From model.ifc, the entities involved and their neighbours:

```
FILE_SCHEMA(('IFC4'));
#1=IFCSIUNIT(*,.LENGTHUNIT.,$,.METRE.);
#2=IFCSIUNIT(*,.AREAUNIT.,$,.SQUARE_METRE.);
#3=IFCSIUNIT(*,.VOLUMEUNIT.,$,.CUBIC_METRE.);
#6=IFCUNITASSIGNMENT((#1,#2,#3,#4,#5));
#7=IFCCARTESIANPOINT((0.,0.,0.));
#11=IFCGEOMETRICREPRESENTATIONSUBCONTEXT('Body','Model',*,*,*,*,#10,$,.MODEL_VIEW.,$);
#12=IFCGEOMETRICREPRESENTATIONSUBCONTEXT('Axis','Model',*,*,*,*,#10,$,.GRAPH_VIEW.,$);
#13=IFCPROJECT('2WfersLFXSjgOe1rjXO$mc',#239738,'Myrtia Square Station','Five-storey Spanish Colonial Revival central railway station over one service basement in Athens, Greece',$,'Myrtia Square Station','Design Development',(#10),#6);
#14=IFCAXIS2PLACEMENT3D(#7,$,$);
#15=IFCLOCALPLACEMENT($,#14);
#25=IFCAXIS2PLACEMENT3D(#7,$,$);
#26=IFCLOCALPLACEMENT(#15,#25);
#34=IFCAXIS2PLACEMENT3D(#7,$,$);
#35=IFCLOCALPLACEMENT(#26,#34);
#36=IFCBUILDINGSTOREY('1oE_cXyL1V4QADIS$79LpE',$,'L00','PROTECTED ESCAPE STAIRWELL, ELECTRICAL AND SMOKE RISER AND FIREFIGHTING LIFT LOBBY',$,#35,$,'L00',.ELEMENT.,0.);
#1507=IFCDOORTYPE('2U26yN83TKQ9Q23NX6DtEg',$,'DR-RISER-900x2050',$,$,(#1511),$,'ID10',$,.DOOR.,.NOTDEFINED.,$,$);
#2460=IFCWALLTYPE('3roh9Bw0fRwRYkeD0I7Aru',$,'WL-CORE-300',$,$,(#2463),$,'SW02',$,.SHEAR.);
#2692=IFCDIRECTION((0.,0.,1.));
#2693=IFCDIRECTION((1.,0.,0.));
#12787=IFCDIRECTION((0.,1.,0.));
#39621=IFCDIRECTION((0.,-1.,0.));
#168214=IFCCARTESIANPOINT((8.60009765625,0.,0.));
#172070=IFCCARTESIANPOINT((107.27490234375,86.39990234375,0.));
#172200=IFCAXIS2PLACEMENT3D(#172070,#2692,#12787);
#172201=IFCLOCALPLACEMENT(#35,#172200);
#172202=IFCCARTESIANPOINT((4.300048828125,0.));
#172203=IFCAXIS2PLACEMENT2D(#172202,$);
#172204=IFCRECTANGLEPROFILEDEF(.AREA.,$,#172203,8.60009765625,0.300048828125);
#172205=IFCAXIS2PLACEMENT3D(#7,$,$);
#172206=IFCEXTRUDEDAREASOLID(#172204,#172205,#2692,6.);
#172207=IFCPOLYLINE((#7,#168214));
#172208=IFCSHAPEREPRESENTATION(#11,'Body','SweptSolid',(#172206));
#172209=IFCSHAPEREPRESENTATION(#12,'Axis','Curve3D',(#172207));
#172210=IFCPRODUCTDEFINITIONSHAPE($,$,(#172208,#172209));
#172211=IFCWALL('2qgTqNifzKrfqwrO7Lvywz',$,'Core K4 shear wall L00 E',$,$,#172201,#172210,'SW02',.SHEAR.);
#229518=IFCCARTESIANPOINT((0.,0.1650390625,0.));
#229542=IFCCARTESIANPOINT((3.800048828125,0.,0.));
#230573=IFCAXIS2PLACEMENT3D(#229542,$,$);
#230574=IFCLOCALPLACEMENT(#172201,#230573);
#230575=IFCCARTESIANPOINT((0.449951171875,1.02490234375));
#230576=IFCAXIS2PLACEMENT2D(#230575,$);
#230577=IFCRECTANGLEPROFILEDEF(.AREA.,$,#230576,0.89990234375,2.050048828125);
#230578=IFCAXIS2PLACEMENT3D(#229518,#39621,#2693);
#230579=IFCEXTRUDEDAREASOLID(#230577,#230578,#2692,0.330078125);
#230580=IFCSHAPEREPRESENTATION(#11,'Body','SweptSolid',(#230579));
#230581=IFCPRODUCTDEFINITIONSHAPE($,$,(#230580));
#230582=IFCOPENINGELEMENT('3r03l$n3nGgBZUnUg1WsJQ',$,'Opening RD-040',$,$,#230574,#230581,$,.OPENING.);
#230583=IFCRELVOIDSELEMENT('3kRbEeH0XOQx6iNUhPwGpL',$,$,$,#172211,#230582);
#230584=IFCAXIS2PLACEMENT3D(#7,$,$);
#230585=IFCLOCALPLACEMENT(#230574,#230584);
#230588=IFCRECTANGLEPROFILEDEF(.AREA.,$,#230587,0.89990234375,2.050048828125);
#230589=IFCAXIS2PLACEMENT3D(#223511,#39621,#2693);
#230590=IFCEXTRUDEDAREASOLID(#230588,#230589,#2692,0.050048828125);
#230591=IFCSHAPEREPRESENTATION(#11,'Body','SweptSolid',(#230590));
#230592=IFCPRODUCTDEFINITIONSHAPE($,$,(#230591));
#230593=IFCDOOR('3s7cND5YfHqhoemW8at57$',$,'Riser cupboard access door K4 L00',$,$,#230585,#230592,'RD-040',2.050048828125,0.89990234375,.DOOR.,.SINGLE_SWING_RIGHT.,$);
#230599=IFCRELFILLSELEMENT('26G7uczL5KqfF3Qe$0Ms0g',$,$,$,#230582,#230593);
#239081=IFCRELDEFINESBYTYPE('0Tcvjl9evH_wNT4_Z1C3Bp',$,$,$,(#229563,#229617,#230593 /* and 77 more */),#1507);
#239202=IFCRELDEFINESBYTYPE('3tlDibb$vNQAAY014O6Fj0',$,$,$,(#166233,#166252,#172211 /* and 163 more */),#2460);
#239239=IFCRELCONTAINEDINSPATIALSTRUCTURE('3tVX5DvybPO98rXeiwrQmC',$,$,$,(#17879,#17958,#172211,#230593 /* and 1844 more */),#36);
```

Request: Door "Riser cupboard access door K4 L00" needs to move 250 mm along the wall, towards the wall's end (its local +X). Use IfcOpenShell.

```python
import ifcopenshell
import ifcopenshell.api.geometry
import ifcopenshell.util.placement
import ifcopenshell.util.unit

model = ifcopenshell.open("model.ifc")
unit_scale = ifcopenshell.util.unit.calculate_unit_scale(model)

door = model.by_id(230593)
opening = door.FillsVoids[0].RelatingOpeningElement
wall = opening.VoidsElements[0].RelatingBuildingElement

wall_matrix = ifcopenshell.util.placement.get_local_placement(wall.ObjectPlacement)
shift = wall_matrix[:3, 0] * 0.25 / unit_scale
before = ifcopenshell.util.placement.get_local_placement(door.ObjectPlacement)[:3, 3].copy()

# The door is placed relative to its opening, so it follows when the opening moves.
matrix = ifcopenshell.util.placement.get_local_placement(opening.ObjectPlacement)
matrix[:3, 3] += shift
ifcopenshell.api.geometry.edit_object_placement(
    model, product=opening, matrix=matrix, is_si=False, should_transform_children=True
)

after = ifcopenshell.util.placement.get_local_placement(door.ObjectPlacement)[:3, 3]
print("door moved by", (after - before).round(3) + 0.0)

model.write("model_v2.ifc")
```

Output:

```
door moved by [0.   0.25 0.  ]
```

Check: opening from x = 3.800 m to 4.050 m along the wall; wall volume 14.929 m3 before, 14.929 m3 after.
